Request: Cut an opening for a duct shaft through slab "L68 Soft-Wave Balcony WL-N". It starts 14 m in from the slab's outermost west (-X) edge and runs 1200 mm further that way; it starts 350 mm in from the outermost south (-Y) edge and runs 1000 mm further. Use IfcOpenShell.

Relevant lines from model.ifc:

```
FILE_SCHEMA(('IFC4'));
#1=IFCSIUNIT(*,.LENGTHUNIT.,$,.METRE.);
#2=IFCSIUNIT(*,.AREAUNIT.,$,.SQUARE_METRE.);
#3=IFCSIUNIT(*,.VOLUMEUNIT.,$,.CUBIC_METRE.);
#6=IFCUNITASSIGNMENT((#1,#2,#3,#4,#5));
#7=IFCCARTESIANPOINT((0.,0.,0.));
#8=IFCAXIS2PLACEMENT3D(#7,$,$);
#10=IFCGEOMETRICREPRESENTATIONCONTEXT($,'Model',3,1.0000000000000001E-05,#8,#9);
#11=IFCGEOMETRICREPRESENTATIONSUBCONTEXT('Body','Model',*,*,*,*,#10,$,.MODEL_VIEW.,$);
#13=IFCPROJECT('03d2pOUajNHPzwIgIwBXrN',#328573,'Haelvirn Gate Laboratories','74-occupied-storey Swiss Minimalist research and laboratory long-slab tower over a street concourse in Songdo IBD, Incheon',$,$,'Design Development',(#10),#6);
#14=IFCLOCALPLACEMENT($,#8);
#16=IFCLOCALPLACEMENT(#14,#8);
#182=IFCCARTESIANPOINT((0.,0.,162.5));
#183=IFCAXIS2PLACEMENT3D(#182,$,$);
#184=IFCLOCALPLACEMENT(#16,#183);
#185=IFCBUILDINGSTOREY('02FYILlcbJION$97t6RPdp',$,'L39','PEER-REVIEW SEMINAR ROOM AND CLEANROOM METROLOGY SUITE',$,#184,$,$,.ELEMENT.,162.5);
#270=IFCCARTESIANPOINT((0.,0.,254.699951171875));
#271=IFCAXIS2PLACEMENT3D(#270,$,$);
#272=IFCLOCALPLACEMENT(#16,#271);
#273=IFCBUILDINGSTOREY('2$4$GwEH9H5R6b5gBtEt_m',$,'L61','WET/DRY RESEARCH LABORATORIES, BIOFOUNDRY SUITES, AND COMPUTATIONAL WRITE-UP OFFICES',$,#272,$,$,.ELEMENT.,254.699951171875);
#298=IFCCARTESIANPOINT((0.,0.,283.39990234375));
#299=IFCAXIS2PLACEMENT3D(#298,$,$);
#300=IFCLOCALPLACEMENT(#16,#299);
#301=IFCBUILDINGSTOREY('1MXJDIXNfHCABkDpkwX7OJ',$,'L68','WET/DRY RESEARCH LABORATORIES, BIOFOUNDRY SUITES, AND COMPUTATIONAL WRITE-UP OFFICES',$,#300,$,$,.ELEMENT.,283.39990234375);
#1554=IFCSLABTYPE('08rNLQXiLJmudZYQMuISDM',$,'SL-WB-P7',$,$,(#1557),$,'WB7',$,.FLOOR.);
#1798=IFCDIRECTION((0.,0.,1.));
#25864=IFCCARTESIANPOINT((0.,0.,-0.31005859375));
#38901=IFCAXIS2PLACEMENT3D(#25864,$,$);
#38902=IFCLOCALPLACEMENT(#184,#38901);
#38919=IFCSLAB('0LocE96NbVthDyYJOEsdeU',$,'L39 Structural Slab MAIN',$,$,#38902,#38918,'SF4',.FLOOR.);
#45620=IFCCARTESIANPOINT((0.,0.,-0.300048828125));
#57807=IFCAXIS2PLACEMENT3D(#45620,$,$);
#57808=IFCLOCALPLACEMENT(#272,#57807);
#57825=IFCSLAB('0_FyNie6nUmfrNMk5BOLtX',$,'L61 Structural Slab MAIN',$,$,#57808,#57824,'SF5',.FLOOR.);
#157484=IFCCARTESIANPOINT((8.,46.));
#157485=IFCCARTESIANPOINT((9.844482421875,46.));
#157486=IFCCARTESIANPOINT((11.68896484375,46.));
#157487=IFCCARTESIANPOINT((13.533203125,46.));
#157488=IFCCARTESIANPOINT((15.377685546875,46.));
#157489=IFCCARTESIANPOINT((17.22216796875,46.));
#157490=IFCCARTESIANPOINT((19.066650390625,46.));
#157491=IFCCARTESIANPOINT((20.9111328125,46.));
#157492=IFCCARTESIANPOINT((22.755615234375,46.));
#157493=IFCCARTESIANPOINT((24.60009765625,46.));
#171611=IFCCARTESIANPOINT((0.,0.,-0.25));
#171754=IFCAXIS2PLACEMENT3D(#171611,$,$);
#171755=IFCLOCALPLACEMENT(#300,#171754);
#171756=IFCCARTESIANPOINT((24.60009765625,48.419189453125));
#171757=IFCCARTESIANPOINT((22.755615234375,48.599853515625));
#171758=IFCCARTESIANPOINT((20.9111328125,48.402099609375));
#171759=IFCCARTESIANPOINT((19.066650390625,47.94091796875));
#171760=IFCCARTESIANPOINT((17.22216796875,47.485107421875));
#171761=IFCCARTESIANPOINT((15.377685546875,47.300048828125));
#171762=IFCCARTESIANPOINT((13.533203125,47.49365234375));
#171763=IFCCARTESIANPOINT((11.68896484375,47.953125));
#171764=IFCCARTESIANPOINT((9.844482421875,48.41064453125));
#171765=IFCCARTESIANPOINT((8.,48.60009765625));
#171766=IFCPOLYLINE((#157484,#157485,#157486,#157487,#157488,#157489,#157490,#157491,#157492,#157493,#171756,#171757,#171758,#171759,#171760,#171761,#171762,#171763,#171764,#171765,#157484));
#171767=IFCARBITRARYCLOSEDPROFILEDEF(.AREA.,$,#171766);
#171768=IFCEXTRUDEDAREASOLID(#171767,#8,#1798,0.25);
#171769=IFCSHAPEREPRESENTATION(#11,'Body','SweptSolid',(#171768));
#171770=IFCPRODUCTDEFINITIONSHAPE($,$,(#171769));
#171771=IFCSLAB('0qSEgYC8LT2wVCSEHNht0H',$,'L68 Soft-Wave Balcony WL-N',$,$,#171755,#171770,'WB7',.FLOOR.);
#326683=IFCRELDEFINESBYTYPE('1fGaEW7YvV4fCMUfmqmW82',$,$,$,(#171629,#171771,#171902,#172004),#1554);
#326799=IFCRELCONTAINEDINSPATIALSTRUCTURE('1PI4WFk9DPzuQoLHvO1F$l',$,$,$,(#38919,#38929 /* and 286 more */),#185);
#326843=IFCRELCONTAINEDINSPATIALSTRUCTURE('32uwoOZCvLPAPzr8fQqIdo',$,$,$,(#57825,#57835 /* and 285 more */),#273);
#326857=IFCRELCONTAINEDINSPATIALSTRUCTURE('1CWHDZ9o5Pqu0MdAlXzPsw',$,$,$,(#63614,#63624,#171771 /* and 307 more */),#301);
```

```python
import numpy as np
import ifcopenshell
import ifcopenshell.api.feature
import ifcopenshell.api.geometry
import ifcopenshell.api.root
import ifcopenshell.geom
import ifcopenshell.util.placement
import ifcopenshell.util.representation
import ifcopenshell.util.shape
import ifcopenshell.util.unit

model = ifcopenshell.open("model.ifc")
unit_scale = ifcopenshell.util.unit.calculate_unit_scale(model)
settings = ifcopenshell.geom.settings()


def volume(element):
    """Net volume in cubic metres, openings subtracted."""
    shape = ifcopenshell.geom.create_shape(settings, element)
    return ifcopenshell.util.shape.get_volume(shape.geometry)


slab = model.by_guid("0qSEgYC8LT2wVCSEHNht0H")
before = volume(slab)

# Extent in the slab's own axes, in metres. The edges named are its -X and -Y sides.
slab_shape = ifcopenshell.geom.create_shape(settings, slab)
vertices = ifcopenshell.util.shape.get_vertices(slab_shape.geometry)
x_min, y_min, bottom = vertices.min(axis=0)
top = vertices[:, 2].max()

opening = ifcopenshell.api.root.create_entity(model, ifc_class="IfcOpeningElement", name="Duct shaft opening", predefined_type="OPENING")
context = ifcopenshell.util.representation.get_context(model, "Model", "Body", "MODEL_VIEW")
width, depth = 1.2, 1
outline = [(0.0, 0.0), (width, 0.0), (width, depth), (0.0, depth), (0.0, 0.0)]
# Overshoot both faces by 50 mm so the cut is clean.
shape = ifcopenshell.api.geometry.add_slab_representation(
    model, context=context, depth=top - bottom + 0.1, polyline=outline
)
ifcopenshell.api.geometry.assign_representation(model, product=opening, representation=shape)

matrix = ifcopenshell.util.placement.get_local_placement(slab.ObjectPlacement)
matrix[:, 3] = matrix @ np.append(np.array([x_min + 14, y_min + 0.35, bottom - 0.05]) / unit_scale, 1.0)
ifcopenshell.api.geometry.edit_object_placement(model, product=opening, matrix=matrix, is_si=False)
ifcopenshell.api.feature.add_feature(model, feature=opening, element=slab)

after = volume(slab)

print(f"slab volume {before:.3f} -> {after:.3f} m3")

model.write("model_rev.ifc")
```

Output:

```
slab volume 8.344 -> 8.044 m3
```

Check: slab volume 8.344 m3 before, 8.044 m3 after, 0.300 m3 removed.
